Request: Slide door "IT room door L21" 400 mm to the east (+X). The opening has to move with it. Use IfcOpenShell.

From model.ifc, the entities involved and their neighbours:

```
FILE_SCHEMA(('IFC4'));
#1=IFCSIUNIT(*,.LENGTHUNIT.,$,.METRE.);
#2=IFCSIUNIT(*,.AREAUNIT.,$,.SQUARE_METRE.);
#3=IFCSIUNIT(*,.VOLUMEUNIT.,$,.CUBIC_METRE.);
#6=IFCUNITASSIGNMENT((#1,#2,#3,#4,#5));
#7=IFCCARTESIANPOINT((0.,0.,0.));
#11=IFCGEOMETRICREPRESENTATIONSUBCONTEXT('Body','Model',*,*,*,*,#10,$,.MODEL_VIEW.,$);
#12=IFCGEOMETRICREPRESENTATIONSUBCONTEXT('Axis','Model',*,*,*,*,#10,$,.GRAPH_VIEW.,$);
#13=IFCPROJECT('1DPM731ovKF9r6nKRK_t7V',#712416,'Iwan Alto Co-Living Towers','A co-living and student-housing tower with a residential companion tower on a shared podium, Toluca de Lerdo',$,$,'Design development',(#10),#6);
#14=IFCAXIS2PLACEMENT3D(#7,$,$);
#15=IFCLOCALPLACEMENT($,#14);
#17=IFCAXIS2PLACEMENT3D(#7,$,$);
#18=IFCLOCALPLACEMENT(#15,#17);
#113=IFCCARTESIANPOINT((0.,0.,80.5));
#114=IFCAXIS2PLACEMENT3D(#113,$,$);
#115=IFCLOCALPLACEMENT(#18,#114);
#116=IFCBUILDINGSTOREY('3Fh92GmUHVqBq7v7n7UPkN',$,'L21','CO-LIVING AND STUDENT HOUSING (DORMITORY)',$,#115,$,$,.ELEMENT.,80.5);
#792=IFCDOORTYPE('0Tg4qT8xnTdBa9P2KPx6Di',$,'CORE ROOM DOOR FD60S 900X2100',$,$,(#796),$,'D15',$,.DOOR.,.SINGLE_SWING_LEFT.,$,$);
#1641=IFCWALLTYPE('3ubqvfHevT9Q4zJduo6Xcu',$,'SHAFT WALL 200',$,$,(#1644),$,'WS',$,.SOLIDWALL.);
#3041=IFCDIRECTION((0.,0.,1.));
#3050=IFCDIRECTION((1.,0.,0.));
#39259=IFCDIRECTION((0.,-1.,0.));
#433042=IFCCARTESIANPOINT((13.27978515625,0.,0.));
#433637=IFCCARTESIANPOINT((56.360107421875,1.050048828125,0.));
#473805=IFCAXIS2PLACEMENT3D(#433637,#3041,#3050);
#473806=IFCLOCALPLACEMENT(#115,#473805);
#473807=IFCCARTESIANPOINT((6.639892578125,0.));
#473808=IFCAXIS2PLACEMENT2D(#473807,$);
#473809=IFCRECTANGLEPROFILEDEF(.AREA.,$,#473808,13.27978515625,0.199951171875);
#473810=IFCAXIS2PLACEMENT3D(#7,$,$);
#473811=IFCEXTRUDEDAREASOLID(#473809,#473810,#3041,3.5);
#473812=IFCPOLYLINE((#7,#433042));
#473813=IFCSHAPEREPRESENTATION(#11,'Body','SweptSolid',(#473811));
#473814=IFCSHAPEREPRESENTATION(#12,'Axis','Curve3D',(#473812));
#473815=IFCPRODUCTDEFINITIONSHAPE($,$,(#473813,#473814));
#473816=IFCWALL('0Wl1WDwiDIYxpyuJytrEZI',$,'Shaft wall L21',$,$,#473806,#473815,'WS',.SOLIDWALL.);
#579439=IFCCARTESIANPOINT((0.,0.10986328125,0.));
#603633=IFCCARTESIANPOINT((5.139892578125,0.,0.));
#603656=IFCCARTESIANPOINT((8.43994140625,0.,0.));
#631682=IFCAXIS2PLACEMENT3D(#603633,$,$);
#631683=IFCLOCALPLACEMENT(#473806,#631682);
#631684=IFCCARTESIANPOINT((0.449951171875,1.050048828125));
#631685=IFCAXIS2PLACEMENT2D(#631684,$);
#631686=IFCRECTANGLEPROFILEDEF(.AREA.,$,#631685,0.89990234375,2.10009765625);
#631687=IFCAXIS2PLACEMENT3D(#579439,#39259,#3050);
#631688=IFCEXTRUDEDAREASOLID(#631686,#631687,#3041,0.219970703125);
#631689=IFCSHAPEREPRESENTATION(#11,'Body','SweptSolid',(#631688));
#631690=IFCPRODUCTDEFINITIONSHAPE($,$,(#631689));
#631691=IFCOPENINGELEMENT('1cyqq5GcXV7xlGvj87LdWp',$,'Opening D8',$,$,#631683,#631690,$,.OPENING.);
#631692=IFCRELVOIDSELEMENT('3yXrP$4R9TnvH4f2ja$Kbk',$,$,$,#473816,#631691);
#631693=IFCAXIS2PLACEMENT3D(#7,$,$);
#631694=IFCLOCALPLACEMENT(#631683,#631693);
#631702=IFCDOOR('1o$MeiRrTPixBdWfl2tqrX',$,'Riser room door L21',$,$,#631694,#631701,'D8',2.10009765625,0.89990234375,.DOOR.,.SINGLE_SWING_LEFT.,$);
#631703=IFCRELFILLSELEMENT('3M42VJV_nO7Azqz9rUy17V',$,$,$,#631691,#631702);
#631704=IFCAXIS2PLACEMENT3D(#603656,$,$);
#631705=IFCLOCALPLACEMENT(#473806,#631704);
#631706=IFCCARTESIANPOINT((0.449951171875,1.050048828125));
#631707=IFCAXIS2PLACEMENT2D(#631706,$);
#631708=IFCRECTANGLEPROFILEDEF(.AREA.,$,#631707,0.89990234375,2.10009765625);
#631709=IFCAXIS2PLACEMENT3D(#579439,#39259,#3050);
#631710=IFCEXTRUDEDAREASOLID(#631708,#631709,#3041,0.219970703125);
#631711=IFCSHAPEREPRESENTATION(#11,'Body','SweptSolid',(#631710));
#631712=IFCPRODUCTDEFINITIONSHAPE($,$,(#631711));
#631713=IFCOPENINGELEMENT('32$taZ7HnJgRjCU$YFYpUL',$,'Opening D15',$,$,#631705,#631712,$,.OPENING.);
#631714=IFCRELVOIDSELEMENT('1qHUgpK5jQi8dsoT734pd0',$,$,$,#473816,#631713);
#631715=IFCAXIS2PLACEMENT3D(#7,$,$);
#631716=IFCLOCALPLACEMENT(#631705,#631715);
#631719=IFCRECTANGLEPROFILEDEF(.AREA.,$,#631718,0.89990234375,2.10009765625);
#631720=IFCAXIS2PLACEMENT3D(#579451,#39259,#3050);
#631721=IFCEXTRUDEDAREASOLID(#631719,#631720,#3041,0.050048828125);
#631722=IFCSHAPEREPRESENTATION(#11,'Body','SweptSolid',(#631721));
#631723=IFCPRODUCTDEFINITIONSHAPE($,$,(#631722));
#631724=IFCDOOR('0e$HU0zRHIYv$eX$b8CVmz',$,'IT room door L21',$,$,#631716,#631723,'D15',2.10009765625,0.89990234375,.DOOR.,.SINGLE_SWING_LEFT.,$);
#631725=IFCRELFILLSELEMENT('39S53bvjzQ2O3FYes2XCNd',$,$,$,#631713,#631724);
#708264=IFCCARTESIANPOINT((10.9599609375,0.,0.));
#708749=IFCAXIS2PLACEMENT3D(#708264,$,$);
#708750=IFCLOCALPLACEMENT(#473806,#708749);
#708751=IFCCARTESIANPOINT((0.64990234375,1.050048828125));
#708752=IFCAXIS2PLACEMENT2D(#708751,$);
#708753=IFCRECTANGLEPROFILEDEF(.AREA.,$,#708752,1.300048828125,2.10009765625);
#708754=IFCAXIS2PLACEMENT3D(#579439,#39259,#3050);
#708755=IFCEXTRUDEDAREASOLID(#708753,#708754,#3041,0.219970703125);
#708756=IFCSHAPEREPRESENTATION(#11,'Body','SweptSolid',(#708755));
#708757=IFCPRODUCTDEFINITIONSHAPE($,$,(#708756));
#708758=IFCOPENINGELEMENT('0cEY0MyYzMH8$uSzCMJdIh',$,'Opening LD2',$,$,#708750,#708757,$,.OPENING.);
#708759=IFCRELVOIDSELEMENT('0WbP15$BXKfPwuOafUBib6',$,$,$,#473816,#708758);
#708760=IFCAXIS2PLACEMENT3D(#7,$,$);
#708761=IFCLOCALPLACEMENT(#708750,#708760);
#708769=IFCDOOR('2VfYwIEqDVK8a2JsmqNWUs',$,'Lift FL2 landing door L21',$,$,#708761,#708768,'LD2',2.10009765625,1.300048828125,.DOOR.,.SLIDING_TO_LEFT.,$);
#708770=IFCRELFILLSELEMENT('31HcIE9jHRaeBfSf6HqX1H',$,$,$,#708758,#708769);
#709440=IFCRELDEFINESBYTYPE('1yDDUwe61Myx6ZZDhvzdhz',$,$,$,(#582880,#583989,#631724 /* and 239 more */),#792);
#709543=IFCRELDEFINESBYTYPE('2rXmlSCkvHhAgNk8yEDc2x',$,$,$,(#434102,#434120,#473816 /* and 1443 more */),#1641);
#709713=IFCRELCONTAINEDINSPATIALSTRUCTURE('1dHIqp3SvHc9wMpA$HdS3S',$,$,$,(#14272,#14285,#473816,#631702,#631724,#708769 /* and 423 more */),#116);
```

```python
import ifcopenshell
import ifcopenshell.api.geometry
import ifcopenshell.util.placement

model = ifcopenshell.open("model.ifc")

door = model.by_id(631724)
opening = door.FillsVoids[0].RelatingOpeningElement
wall = opening.VoidsElements[0].RelatingBuildingElement

wall_matrix = ifcopenshell.util.placement.get_local_placement(wall.ObjectPlacement)
shift = wall_matrix[:3, 0] * 0.4
before = ifcopenshell.util.placement.get_local_placement(door.ObjectPlacement)[:3, 3].copy()

# The door is placed relative to its opening, so it follows when the opening moves.
matrix = ifcopenshell.util.placement.get_local_placement(opening.ObjectPlacement)
matrix[:3, 3] += shift
ifcopenshell.api.geometry.edit_object_placement(
    model, product=opening, matrix=matrix, is_si=False, should_transform_children=True
)

after = ifcopenshell.util.placement.get_local_placement(door.ObjectPlacement)[:3, 3]
print("door moved by", (after - before).round(3) + 0.0)

model.write("model_v2.ifc")
```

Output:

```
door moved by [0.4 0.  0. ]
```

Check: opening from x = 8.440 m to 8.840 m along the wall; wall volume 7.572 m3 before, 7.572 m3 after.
